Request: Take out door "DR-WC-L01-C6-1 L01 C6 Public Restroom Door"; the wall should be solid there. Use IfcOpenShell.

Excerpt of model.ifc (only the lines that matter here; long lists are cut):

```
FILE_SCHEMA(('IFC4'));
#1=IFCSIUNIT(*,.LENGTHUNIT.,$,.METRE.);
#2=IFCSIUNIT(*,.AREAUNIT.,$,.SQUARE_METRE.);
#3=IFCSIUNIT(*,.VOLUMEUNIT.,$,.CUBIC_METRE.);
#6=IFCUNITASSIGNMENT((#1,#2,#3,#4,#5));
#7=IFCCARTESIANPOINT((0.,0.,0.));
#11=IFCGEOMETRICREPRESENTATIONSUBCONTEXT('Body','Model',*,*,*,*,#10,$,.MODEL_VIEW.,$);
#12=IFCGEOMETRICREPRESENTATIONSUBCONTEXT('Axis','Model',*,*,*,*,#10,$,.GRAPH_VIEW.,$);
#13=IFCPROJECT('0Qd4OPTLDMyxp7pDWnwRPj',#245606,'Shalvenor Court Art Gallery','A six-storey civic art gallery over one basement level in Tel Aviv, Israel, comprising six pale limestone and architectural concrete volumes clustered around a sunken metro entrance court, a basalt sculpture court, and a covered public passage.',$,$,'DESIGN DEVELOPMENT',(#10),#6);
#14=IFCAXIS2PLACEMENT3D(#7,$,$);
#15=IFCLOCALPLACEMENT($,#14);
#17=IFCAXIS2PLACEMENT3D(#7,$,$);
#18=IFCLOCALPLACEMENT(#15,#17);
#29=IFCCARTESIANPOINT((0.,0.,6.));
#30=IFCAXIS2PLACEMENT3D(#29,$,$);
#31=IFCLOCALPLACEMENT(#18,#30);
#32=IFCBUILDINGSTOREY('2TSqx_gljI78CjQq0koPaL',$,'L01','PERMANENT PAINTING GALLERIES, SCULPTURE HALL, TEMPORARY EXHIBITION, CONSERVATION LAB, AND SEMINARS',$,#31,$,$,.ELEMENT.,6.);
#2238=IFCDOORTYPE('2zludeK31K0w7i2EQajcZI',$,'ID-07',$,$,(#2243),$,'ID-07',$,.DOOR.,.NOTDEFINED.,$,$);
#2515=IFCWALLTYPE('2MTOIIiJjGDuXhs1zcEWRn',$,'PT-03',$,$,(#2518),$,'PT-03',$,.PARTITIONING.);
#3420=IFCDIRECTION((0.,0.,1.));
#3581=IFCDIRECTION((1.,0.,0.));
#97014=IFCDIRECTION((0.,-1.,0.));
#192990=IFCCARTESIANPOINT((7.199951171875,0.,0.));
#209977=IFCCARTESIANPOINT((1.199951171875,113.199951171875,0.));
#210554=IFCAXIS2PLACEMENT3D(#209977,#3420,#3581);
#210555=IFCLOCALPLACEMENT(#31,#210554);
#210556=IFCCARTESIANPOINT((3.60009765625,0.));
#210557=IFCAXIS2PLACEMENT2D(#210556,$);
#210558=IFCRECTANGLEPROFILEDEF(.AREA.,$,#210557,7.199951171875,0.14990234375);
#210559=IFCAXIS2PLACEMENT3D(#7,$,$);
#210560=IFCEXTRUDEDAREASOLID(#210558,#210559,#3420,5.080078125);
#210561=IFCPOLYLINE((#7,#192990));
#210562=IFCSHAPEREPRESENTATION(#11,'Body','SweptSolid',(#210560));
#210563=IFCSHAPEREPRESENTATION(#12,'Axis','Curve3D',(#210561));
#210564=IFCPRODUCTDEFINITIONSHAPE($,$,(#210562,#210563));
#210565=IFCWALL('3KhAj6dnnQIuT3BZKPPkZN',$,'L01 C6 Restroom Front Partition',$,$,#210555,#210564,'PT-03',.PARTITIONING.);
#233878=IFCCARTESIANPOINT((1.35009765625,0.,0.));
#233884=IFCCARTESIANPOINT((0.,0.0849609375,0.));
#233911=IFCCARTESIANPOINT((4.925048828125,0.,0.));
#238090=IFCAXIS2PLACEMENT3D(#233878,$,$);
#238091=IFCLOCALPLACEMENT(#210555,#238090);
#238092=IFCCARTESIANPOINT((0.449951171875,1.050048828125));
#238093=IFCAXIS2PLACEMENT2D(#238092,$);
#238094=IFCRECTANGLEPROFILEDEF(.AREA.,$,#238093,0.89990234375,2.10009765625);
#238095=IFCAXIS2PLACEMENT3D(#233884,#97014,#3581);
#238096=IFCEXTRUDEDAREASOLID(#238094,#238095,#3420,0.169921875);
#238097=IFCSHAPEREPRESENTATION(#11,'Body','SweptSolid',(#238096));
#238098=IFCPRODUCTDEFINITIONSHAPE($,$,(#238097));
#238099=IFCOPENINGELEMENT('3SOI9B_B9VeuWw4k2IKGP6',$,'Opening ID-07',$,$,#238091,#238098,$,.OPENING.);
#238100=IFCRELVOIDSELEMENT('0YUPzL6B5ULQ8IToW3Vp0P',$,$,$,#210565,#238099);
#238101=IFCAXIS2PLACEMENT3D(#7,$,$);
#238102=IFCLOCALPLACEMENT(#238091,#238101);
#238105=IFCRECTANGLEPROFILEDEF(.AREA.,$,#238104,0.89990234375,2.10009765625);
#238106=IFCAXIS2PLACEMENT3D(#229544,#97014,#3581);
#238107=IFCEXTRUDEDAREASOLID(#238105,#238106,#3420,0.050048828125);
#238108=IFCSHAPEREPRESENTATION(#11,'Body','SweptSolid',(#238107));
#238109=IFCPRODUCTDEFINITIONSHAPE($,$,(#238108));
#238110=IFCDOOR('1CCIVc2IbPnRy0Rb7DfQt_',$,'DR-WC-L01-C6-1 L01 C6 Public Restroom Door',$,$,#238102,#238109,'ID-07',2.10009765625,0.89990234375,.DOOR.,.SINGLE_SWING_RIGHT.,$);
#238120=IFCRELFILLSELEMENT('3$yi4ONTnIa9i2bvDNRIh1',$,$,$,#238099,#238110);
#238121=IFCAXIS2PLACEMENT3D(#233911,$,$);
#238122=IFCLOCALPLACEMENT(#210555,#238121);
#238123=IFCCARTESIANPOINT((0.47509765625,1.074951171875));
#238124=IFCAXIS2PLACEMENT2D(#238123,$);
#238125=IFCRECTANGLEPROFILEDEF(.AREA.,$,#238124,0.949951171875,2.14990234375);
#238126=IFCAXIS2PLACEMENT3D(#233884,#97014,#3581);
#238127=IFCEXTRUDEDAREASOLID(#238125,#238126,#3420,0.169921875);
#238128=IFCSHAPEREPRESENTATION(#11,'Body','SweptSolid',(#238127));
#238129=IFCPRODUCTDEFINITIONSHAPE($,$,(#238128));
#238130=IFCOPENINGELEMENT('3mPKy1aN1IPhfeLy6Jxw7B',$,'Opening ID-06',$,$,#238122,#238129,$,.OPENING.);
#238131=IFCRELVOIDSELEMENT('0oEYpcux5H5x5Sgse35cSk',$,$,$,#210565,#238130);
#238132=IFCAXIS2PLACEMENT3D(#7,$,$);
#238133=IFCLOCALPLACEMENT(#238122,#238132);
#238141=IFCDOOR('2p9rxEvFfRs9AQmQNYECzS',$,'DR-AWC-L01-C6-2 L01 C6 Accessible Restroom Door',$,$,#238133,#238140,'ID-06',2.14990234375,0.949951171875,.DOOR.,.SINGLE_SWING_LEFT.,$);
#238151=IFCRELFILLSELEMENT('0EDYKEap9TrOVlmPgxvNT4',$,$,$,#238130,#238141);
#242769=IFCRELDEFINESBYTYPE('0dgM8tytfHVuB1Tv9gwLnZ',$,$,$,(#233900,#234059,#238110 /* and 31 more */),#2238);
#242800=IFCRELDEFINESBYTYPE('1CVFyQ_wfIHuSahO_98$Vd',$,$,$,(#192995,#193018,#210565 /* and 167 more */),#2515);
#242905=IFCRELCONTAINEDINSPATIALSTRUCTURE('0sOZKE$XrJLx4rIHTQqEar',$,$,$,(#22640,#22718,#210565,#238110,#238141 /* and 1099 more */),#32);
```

```python
import ifcopenshell
import ifcopenshell.api.feature
import ifcopenshell.api.root
import ifcopenshell.geom
import ifcopenshell.util.shape

model = ifcopenshell.open("model.ifc")
settings = ifcopenshell.geom.settings()


def volume(element):
    """Net volume in cubic metres, openings subtracted."""
    shape = ifcopenshell.geom.create_shape(settings, element)
    return ifcopenshell.util.shape.get_volume(shape.geometry)


door = model.by_guid("1CCIVc2IbPnRy0Rb7DfQt_")
opening = door.FillsVoids[0].RelatingOpeningElement
wall = opening.VoidsElements[0].RelatingBuildingElement
before = volume(wall)

ifcopenshell.api.root.remove_product(model, product=door)
ifcopenshell.api.feature.remove_feature(model, feature=opening)

after = volume(wall)

print(f"wall volume {before:.3f} -> {after:.3f} m3")

model.write("model-out.ifc")
```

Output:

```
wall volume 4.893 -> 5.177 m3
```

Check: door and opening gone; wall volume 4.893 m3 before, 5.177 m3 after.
